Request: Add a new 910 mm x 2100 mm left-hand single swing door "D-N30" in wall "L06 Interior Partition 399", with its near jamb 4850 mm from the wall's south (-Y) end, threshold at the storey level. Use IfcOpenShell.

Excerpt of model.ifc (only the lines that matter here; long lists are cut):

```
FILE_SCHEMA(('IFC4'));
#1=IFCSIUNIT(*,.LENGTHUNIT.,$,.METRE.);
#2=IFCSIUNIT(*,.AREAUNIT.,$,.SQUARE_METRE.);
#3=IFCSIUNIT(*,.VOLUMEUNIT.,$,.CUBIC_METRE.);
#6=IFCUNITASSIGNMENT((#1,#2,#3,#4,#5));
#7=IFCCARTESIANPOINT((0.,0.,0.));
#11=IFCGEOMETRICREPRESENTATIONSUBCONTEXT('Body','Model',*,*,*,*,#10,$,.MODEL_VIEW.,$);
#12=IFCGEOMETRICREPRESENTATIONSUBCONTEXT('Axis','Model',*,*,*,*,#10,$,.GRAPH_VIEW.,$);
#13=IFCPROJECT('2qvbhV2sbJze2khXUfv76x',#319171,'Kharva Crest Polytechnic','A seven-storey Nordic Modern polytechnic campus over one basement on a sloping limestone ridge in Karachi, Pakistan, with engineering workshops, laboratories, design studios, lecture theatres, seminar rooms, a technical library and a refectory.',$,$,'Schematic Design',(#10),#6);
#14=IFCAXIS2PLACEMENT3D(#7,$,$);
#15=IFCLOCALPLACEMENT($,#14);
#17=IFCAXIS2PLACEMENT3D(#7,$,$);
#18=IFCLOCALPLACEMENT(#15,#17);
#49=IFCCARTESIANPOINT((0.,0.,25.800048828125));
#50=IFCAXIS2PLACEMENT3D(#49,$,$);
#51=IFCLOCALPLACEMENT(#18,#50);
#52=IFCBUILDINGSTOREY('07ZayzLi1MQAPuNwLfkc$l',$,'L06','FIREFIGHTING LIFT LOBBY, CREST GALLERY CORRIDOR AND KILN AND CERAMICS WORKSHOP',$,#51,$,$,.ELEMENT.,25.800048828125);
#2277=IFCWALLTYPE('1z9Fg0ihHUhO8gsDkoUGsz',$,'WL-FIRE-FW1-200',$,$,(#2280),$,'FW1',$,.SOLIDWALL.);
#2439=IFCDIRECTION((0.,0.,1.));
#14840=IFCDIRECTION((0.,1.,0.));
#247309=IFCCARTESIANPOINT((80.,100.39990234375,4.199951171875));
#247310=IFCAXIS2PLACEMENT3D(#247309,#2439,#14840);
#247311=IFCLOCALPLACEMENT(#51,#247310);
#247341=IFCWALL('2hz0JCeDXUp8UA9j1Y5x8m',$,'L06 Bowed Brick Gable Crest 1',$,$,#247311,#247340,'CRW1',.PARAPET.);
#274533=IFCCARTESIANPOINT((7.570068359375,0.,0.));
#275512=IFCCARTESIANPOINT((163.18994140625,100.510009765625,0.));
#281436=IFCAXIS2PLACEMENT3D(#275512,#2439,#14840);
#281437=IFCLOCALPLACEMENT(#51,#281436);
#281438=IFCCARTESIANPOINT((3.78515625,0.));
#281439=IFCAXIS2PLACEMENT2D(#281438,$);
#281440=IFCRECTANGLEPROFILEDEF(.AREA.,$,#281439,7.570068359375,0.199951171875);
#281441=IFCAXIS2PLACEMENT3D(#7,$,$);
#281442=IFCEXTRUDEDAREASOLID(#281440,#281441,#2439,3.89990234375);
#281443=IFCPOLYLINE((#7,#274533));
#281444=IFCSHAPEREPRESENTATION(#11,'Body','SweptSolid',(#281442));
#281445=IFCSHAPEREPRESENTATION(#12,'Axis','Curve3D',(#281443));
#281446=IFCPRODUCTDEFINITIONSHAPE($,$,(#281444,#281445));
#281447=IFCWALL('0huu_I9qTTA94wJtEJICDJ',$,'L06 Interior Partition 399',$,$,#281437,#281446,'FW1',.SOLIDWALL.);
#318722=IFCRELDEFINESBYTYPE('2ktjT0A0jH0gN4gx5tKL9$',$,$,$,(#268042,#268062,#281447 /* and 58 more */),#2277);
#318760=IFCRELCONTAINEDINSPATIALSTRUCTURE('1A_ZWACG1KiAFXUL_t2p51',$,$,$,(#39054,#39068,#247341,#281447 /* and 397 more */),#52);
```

```python
import numpy as np
import ifcopenshell
import ifcopenshell.api.feature
import ifcopenshell.api.geometry
import ifcopenshell.api.root
import ifcopenshell.api.spatial
import ifcopenshell.geom
import ifcopenshell.util.element
import ifcopenshell.util.placement
import ifcopenshell.util.representation
import ifcopenshell.util.shape
import ifcopenshell.util.unit

model = ifcopenshell.open("model.ifc")
unit_scale = ifcopenshell.util.unit.calculate_unit_scale(model)
settings = ifcopenshell.geom.settings()


def volume(element):
    """Net volume in cubic metres, openings subtracted."""
    shape = ifcopenshell.geom.create_shape(settings, element)
    return ifcopenshell.util.shape.get_volume(shape.geometry)


wall = model.by_guid("0huu_I9qTTA94wJtEJICDJ")
storey = ifcopenshell.util.element.get_container(wall, ifc_class="IfcBuildingStorey")
context = ifcopenshell.util.representation.get_context(model, "Model", "Body", "MODEL_VIEW")
before = volume(wall)

width, height, from_end, sill = 0.91, 2.1, 4.85, 0.0  # metres

# The wall runs along its own X axis, and the end named is its -X end.
wall_shape = ifcopenshell.geom.create_shape(settings, wall)
x, y, z = ifcopenshell.util.shape.get_vertices(wall_shape.geometry).T
start = x.min() + from_end
face, thickness = float(y.min()), float(y.max() - y.min())
wall_matrix = ifcopenshell.util.placement.get_local_placement(wall.ObjectPlacement)
level = ifcopenshell.util.placement.get_local_placement(storey.ObjectPlacement)[2, 3]


def in_wall(x, y):
    """Placement at x, y metres in the wall's axes, at sill height."""
    matrix = wall_matrix.copy()
    matrix[:, 3] = wall_matrix @ np.array([x / unit_scale, y / unit_scale, 0.0, 1.0])
    matrix[2, 3] = level + sill / unit_scale
    return matrix


# Opening: a box that overshoots both wall faces by 50 mm.
opening = ifcopenshell.api.root.create_entity(model, ifc_class="IfcOpeningElement", predefined_type="OPENING")
box = ifcopenshell.api.geometry.add_wall_representation(
    model, context=context, length=width, height=height, thickness=thickness + 0.1
)
ifcopenshell.api.geometry.assign_representation(model, product=opening, representation=box)
ifcopenshell.api.geometry.edit_object_placement(model, product=opening, matrix=in_wall(start, face - 0.05), is_si=False)
ifcopenshell.api.feature.add_feature(model, feature=opening, element=wall)

door = ifcopenshell.api.root.create_entity(model, ifc_class="IfcDoor", name="D-N30", predefined_type="DOOR")
door.OverallWidth, door.OverallHeight = width / unit_scale, height / unit_scale
door.OperationType = "SINGLE_SWING_LEFT"
body = ifcopenshell.api.geometry.add_door_representation(
    model,
    context=context,
    overall_width=door.OverallWidth,
    overall_height=door.OverallHeight,
    operation_type="SINGLE_SWING_LEFT",
    lining_properties={"LiningDepth": thickness / unit_scale, "ThresholdDepth": thickness / unit_scale},
)
ifcopenshell.api.geometry.assign_representation(model, product=door, representation=body)
ifcopenshell.api.spatial.assign_container(model, products=[door], relating_structure=storey)
ifcopenshell.api.feature.add_filling(model, opening=opening, element=door)

# The lining spans the wall, so the door starts at the wall face.
ifcopenshell.api.geometry.edit_object_placement(model, product=door, matrix=in_wall(start, face), is_si=False)

after = volume(wall)

print(f"wall volume {before:.3f} -> {after:.3f} m3")

model.write("model_v2.ifc")
```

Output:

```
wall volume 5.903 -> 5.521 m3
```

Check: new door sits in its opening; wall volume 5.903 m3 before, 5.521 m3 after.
